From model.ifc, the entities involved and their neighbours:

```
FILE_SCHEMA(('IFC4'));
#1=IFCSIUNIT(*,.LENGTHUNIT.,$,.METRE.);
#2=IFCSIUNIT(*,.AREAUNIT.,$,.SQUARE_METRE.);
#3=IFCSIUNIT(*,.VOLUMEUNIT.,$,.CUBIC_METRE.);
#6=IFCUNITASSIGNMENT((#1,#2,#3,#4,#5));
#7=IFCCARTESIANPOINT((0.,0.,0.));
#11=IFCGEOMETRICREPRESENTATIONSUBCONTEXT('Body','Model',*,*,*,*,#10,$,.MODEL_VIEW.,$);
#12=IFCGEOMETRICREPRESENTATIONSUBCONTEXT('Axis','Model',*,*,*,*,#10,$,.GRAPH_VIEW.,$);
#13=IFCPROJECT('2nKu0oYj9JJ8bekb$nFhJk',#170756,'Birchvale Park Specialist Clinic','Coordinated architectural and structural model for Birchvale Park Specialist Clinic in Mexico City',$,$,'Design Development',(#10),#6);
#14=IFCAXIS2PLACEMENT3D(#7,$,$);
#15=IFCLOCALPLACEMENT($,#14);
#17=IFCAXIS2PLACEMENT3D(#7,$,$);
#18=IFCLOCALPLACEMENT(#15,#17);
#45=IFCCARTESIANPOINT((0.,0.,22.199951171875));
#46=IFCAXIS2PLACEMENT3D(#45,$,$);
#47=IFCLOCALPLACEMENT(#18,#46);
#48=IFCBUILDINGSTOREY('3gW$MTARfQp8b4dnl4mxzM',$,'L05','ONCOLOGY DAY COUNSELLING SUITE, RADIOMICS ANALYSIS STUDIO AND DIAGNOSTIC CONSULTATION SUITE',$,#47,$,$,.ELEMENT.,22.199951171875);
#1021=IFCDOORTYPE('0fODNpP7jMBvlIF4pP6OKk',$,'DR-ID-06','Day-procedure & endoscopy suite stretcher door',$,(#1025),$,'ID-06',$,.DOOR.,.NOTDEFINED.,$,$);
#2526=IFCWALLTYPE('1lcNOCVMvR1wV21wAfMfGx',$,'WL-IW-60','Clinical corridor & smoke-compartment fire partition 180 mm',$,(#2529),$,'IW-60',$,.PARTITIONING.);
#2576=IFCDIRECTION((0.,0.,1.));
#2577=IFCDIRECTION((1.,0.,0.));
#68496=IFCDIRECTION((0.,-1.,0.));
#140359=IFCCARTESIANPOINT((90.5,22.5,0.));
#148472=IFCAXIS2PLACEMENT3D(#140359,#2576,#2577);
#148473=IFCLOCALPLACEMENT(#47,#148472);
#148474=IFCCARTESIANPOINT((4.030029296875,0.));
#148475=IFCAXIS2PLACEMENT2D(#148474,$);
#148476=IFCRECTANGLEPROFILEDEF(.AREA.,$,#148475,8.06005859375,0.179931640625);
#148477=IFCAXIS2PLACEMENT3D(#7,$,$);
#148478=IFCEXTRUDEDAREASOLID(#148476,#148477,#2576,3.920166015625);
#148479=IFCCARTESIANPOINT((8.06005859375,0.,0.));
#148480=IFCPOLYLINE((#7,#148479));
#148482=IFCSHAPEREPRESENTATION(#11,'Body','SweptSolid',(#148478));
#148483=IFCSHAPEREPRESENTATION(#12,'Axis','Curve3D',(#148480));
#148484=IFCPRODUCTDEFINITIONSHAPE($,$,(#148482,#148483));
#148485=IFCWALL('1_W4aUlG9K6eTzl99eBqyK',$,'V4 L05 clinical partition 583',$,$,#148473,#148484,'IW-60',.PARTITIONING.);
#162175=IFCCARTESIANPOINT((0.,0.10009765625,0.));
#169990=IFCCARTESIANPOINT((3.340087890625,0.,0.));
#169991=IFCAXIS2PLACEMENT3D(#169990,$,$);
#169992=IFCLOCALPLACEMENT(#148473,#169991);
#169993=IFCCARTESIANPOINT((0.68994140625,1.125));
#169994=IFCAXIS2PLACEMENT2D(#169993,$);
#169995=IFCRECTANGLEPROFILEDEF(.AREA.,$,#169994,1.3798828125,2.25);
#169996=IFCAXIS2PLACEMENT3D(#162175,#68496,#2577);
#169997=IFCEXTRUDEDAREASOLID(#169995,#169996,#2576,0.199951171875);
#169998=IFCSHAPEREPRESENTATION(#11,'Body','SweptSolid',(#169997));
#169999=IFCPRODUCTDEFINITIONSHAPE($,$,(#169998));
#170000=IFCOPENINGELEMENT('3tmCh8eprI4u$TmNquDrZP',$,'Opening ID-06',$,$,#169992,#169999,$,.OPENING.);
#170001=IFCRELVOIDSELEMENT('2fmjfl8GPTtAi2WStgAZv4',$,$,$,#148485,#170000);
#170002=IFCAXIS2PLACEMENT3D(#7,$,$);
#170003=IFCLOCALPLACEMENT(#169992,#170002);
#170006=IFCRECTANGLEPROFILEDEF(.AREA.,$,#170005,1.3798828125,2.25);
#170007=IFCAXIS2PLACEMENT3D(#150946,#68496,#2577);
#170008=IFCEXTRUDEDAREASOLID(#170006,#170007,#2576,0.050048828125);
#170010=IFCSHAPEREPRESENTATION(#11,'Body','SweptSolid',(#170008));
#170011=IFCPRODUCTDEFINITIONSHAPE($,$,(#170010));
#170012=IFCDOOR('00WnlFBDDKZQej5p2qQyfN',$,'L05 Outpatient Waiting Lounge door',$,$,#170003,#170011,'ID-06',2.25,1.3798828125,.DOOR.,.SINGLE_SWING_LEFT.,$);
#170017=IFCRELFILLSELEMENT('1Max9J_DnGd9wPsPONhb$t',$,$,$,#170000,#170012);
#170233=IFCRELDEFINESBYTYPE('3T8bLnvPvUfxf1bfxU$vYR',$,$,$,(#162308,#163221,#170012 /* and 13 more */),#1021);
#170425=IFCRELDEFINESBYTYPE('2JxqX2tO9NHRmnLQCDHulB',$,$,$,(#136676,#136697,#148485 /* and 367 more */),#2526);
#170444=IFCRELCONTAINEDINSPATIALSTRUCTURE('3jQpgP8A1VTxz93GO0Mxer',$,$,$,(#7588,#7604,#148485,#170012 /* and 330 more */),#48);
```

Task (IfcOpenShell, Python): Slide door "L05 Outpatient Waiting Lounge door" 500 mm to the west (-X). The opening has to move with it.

```python
import ifcopenshell
import ifcopenshell.api.geometry
import ifcopenshell.util.placement
import ifcopenshell.util.unit

model = ifcopenshell.open("model.ifc")
unit_scale = ifcopenshell.util.unit.calculate_unit_scale(model)

door = model.by_guid("00WnlFBDDKZQej5p2qQyfN")
opening = door.FillsVoids[0].RelatingOpeningElement
wall = opening.VoidsElements[0].RelatingBuildingElement

wall_matrix = ifcopenshell.util.placement.get_local_placement(wall.ObjectPlacement)
shift = wall_matrix[:3, 0] * -0.5 / unit_scale
before = ifcopenshell.util.placement.get_local_placement(door.ObjectPlacement)[:3, 3].copy()

# The door is placed relative to its opening, so it follows when the opening moves.
matrix = ifcopenshell.util.placement.get_local_placement(opening.ObjectPlacement)
matrix[:3, 3] += shift
ifcopenshell.api.geometry.edit_object_placement(
    model, product=opening, matrix=matrix, is_si=False, should_transform_children=True
)

after = ifcopenshell.util.placement.get_local_placement(door.ObjectPlacement)[:3, 3]
print("door moved by", (after - before).round(3) + 0.0)

model.write("model_rev.ifc")
```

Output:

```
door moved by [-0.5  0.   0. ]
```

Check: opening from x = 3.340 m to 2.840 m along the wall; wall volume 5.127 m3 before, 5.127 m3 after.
